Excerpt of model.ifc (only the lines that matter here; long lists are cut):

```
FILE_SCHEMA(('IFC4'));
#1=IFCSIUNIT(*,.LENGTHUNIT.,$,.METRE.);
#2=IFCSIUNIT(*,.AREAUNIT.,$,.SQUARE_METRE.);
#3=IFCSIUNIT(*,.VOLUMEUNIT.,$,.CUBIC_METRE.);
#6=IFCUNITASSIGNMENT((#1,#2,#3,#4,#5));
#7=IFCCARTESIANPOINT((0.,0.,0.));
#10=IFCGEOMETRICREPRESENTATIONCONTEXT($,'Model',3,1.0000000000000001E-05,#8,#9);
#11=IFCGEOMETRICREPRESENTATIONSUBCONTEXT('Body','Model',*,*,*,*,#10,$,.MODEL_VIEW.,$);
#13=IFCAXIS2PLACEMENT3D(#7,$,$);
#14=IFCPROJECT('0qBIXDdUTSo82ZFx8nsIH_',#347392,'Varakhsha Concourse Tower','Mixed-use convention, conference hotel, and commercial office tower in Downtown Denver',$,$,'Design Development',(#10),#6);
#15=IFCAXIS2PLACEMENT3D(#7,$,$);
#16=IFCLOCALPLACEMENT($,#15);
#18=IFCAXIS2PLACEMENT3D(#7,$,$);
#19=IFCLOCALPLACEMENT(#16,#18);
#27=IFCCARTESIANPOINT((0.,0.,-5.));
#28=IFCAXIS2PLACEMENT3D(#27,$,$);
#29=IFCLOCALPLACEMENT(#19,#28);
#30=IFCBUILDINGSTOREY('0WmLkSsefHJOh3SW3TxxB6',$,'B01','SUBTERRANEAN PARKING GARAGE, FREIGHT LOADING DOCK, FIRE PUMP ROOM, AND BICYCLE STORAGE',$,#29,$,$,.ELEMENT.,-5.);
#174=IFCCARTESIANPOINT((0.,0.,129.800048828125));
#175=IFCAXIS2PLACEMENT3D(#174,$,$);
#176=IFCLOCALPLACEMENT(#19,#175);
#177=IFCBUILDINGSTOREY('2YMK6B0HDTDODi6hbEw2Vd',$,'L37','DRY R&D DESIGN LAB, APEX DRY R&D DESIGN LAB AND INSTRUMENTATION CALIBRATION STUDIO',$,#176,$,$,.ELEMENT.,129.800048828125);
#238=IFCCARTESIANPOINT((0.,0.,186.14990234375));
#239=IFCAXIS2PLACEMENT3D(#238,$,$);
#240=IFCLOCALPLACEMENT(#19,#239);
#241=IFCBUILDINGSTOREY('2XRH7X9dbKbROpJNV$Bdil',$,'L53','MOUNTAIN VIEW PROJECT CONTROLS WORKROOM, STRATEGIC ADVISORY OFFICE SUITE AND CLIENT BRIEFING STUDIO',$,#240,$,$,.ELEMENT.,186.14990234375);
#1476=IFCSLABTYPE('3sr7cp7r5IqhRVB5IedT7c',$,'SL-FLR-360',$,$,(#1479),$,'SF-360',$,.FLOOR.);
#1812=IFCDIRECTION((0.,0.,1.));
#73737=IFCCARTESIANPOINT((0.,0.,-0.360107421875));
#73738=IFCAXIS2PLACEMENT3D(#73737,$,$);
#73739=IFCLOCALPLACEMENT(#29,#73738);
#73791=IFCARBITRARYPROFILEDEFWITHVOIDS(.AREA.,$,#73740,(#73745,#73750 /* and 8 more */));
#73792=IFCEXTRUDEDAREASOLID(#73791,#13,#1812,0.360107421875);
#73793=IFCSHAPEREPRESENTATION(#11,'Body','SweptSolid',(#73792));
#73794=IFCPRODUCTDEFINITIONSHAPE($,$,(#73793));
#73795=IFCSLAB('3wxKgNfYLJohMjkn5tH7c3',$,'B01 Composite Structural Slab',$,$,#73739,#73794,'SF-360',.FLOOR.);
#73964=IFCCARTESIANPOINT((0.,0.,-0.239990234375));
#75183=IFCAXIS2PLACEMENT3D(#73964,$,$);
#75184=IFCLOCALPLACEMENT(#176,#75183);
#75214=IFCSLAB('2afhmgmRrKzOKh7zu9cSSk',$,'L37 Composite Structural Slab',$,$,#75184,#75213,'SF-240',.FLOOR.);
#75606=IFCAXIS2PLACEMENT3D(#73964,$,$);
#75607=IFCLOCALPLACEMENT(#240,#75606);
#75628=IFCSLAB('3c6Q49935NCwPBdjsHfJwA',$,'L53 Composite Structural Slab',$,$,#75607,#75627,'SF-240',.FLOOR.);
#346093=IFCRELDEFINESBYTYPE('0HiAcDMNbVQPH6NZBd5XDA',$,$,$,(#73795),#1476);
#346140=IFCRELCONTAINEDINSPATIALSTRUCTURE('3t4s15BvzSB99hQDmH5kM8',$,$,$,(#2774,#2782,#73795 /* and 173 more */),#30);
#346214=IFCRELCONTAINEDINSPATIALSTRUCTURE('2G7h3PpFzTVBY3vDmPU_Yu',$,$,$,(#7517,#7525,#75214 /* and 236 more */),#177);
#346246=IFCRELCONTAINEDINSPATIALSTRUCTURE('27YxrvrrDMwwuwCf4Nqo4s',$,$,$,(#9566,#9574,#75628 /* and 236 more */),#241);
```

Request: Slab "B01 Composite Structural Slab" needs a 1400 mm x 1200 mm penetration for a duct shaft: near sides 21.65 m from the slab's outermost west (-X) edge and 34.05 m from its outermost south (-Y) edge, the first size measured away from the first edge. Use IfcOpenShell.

```python
import numpy as np
import ifcopenshell
import ifcopenshell.api.feature
import ifcopenshell.api.geometry
import ifcopenshell.api.root
import ifcopenshell.geom
import ifcopenshell.util.placement
import ifcopenshell.util.representation
import ifcopenshell.util.shape
import ifcopenshell.util.unit

model = ifcopenshell.open("model.ifc")
unit_scale = ifcopenshell.util.unit.calculate_unit_scale(model)
settings = ifcopenshell.geom.settings()


def volume(element):
    """Net volume in cubic metres, openings subtracted."""
    shape = ifcopenshell.geom.create_shape(settings, element)
    return ifcopenshell.util.shape.get_volume(shape.geometry)


slab = model.by_guid("3wxKgNfYLJohMjkn5tH7c3")
before = volume(slab)

# Extent in the slab's own axes, in metres. The edges named are its -X and -Y sides.
slab_shape = ifcopenshell.geom.create_shape(settings, slab)
vertices = ifcopenshell.util.shape.get_vertices(slab_shape.geometry)
x_min, y_min, bottom = vertices.min(axis=0)
top = vertices[:, 2].max()

opening = ifcopenshell.api.root.create_entity(model, ifc_class="IfcOpeningElement", name="Duct shaft opening", predefined_type="OPENING")
context = ifcopenshell.util.representation.get_context(model, "Model", "Body", "MODEL_VIEW")
width, depth = 1.4, 1.2
outline = [(0.0, 0.0), (width, 0.0), (width, depth), (0.0, depth), (0.0, 0.0)]
# Overshoot both faces by 50 mm so the cut is clean.
shape = ifcopenshell.api.geometry.add_slab_representation(
    model, context=context, depth=top - bottom + 0.1, polyline=outline
)
ifcopenshell.api.geometry.assign_representation(model, product=opening, representation=shape)

matrix = ifcopenshell.util.placement.get_local_placement(slab.ObjectPlacement)
matrix[:, 3] = matrix @ np.append(np.array([x_min + 21.65, y_min + 34.05, bottom - 0.05]) / unit_scale, 1.0)
ifcopenshell.api.geometry.edit_object_placement(model, product=opening, matrix=matrix, is_si=False)
ifcopenshell.api.feature.add_feature(model, feature=opening, element=slab)

after = volume(slab)

print(f"slab volume {before:.3f} -> {after:.3f} m3")

model.write("model_updated.ifc")
```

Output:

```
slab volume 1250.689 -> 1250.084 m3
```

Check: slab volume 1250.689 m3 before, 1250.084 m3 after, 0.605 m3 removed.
